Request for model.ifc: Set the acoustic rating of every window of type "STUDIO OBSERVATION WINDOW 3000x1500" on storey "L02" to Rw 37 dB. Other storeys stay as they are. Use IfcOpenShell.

First a look at what the model holds.

```python
import ifcopenshell
import ifcopenshell.util.element

model = ifcopenshell.open("model.ifc")
print(model.schema)
storey = next(s for s in model.by_type("IfcBuildingStorey") if s.Name == "L02")
windows = [e for e in ifcopenshell.util.element.get_decomposition(storey) if e.is_a("IfcWindow")]
seen = {}
for e in windows:
    element_type = ifcopenshell.util.element.get_type(e)
    key = (element_type.Name if element_type != e and element_type else None, ifcopenshell.util.element.get_pset(e, "Pset_WindowCommon", "AcousticRating"))
    seen[key] = seen.get(key, 0) + 1
for (name, value), count in sorted(seen.items(), key=str):
    print(count, "x", name, "|", value)
```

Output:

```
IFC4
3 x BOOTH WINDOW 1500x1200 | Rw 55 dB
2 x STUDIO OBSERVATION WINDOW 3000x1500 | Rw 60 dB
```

```python
import ifcopenshell
import ifcopenshell.api.pset
import ifcopenshell.util.element

model = ifcopenshell.open("model.ifc")

storey = next(s for s in model.by_type("IfcBuildingStorey") if s.Name == "L02")
windows = [e for e in ifcopenshell.util.element.get_decomposition(storey) if e.is_a("IfcWindow")]

count = 0
for e in windows:
    element_type = ifcopenshell.util.element.get_type(e)
    if element_type in (None, e) or element_type.Name != "STUDIO OBSERVATION WINDOW 3000x1500":
        continue
    found = ifcopenshell.util.element.get_pset(e, "Pset_WindowCommon", should_inherit=False)
    if found:
        pset = model.by_id(found["id"])
        if len(ifcopenshell.util.element.get_elements_by_pset(pset)) > 1:
            pset = ifcopenshell.api.pset.unshare_pset(model, products=[e], pset=pset)[0]
    else:
        pset = ifcopenshell.api.pset.add_pset(model, product=e, name="Pset_WindowCommon")
    ifcopenshell.api.pset.edit_pset(model, pset=pset, properties={"AcousticRating": "Rw 37 dB"})
    count += 1

print(count, "windows updated")

model.write("model_v2.ifc")
```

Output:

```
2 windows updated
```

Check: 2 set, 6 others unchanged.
